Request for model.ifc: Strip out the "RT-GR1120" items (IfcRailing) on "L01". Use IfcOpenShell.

First a look at what the model holds.

```python
import ifcopenshell
import ifcopenshell.util.element

model = ifcopenshell.open("model.ifc")
print(model.schema)
storey = next(s for s in model.by_type("IfcBuildingStorey") if s.Name == "L01")
railings = [e for e in ifcopenshell.util.element.get_decomposition(storey) if e.is_a("IfcRailing")]
seen = {}
for e in railings:
    element_type = ifcopenshell.util.element.get_type(e)
    name = element_type.Name if element_type not in (None, e) else None
    seen[name] = seen.get(name, 0) + 1
for name, count in sorted(seen.items(), key=str):
    print(count, "x", name)
```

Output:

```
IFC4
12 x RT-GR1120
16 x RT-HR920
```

```python
import ifcopenshell
import ifcopenshell.api.root
import ifcopenshell.util.element

model = ifcopenshell.open("model.ifc")

storey = next(s for s in model.by_type("IfcBuildingStorey") if s.Name == "L01")
railings = [e for e in ifcopenshell.util.element.get_decomposition(storey) if e.is_a("IfcRailing")]
targets = [e for e in railings if (t := ifcopenshell.util.element.get_type(e)) not in (None, e) and t.Name == "RT-GR1120"]

for e in targets:
    ifcopenshell.api.root.remove_product(model, product=e)
print(len(targets), "removed")

model.write("model_rev.ifc")
```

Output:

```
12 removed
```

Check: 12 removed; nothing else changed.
